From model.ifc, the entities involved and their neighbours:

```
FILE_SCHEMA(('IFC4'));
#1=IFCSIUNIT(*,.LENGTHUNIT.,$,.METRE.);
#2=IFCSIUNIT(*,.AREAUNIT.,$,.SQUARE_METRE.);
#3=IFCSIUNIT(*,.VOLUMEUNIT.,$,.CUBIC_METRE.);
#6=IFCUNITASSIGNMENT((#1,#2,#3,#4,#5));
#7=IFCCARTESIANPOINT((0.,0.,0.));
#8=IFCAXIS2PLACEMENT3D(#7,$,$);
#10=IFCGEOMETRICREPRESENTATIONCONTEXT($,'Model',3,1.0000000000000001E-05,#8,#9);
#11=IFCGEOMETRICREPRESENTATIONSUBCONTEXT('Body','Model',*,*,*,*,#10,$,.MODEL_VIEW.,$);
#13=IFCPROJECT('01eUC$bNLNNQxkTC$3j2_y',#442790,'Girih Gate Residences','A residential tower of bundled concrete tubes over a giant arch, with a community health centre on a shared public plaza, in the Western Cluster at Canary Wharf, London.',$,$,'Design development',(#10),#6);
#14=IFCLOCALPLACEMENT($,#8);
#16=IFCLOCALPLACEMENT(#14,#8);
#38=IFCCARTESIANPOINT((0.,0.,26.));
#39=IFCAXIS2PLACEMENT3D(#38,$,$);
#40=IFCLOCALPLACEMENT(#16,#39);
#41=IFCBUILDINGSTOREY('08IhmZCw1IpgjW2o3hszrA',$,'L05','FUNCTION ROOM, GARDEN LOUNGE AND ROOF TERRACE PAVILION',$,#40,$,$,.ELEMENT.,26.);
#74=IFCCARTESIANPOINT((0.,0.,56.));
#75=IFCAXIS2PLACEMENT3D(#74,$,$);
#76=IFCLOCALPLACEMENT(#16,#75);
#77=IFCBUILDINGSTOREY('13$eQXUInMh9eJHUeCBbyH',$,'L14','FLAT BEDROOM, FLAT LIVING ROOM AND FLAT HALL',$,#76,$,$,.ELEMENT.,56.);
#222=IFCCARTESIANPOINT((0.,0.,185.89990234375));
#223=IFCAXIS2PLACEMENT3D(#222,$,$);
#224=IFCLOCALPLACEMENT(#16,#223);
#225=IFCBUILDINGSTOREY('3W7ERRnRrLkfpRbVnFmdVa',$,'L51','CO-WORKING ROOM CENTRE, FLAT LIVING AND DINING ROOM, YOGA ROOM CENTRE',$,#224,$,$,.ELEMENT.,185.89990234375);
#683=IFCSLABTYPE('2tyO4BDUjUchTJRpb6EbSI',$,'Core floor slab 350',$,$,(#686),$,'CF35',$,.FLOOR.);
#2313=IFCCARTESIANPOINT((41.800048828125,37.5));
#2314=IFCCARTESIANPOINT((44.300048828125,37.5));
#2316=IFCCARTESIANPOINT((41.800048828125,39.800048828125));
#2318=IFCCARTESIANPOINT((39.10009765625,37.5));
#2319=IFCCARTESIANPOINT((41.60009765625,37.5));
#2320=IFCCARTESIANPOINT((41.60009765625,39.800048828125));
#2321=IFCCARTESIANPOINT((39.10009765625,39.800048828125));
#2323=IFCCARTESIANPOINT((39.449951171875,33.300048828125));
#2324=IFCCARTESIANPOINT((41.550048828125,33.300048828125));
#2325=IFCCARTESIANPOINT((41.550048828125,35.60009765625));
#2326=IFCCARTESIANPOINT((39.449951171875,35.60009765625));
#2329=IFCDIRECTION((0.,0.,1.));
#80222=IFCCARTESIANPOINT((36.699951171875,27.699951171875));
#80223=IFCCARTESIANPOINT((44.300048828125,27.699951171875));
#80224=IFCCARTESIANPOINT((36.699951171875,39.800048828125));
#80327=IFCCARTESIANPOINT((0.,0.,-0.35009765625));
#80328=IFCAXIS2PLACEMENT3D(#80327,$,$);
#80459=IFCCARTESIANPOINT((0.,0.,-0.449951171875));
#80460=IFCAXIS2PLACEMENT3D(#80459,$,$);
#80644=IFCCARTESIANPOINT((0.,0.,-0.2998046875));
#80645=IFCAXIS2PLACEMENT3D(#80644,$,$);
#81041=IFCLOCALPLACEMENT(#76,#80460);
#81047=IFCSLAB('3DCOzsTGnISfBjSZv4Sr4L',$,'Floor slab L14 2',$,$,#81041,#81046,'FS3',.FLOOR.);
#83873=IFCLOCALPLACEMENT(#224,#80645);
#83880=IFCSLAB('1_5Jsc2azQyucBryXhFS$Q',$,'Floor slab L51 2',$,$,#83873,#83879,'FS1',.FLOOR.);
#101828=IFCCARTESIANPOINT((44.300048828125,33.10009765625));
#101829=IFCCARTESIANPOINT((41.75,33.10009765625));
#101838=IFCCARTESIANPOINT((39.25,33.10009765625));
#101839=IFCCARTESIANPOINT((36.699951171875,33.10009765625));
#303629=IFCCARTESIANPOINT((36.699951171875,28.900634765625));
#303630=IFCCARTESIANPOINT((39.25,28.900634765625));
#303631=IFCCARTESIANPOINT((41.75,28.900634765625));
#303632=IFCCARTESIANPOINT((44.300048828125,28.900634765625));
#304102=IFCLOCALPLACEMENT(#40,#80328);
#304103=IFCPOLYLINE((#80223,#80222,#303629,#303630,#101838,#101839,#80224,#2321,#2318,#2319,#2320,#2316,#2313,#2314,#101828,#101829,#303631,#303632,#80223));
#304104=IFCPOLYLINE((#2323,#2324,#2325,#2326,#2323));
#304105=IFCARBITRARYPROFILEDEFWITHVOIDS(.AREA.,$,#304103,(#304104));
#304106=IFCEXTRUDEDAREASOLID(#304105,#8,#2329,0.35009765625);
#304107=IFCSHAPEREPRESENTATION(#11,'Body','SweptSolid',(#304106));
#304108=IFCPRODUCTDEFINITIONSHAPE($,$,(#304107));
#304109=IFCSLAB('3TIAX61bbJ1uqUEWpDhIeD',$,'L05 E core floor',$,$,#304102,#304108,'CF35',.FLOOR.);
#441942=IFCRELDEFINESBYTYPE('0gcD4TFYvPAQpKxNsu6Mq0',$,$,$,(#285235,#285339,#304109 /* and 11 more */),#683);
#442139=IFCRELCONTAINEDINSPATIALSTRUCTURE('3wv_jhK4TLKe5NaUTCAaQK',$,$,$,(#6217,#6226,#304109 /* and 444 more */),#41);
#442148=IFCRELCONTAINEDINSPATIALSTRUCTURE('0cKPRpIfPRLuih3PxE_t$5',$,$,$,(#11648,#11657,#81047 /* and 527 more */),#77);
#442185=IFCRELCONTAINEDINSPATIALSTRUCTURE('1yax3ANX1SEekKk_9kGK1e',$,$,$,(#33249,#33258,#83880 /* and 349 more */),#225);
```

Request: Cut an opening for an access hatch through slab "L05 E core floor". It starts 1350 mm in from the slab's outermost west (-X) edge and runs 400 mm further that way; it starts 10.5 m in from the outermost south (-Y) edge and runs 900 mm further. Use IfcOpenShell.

```python
import numpy as np
import ifcopenshell
import ifcopenshell.api.feature
import ifcopenshell.api.geometry
import ifcopenshell.api.root
import ifcopenshell.geom
import ifcopenshell.util.placement
import ifcopenshell.util.representation
import ifcopenshell.util.shape
import ifcopenshell.util.unit

model = ifcopenshell.open("model.ifc")
unit_scale = ifcopenshell.util.unit.calculate_unit_scale(model)
settings = ifcopenshell.geom.settings()


def volume(element):
    """Net volume in cubic metres, openings subtracted."""
    shape = ifcopenshell.geom.create_shape(settings, element)
    return ifcopenshell.util.shape.get_volume(shape.geometry)


slab = model.by_guid("3TIAX61bbJ1uqUEWpDhIeD")
before = volume(slab)

# Extent in the slab's own axes, in metres. The edges named are its -X and -Y sides.
slab_shape = ifcopenshell.geom.create_shape(settings, slab)
vertices = ifcopenshell.util.shape.get_vertices(slab_shape.geometry)
x_min, y_min, bottom = vertices.min(axis=0)
top = vertices[:, 2].max()

opening = ifcopenshell.api.root.create_entity(model, ifc_class="IfcOpeningElement", name="Access hatch opening", predefined_type="OPENING")
context = ifcopenshell.util.representation.get_context(model, "Model", "Body", "MODEL_VIEW")
width, depth = 0.4, 0.9
outline = [(0.0, 0.0), (width, 0.0), (width, depth), (0.0, depth), (0.0, 0.0)]
# Overshoot both faces by 50 mm so the cut is clean.
shape = ifcopenshell.api.geometry.add_slab_representation(
    model, context=context, depth=top - bottom + 0.1, polyline=outline
)
ifcopenshell.api.geometry.assign_representation(model, product=opening, representation=shape)

matrix = ifcopenshell.util.placement.get_local_placement(slab.ObjectPlacement)
matrix[:, 3] = matrix @ np.append(np.array([x_min + 1.35, y_min + 10.5, bottom - 0.05]) / unit_scale, 1.0)
ifcopenshell.api.geometry.edit_object_placement(model, product=opening, matrix=matrix, is_si=False)
ifcopenshell.api.feature.add_feature(model, feature=opening, element=slab)

after = volume(slab)

print(f"slab volume {before:.3f} -> {after:.3f} m3")

model.write("model_edited.ifc")
```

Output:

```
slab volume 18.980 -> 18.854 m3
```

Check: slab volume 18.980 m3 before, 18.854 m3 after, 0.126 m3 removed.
